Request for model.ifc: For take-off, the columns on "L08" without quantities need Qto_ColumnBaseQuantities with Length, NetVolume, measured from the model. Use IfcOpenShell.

First a look at what the model holds.

```python
import ifcopenshell
import ifcopenshell.util.element
import ifcopenshell.util.unit

model = ifcopenshell.open("model.ifc")
print(model.schema)
for unit_type in ("LENGTHUNIT", "AREAUNIT", "VOLUMEUNIT"):
    print(unit_type, ifcopenshell.util.unit.calculate_unit_scale(model, unit_type))
storey = next(s for s in model.by_type("IfcBuildingStorey") if s.Name == "L08")
columns = [e for e in ifcopenshell.util.element.get_decomposition(storey) if e.is_a("IfcColumn")]
for e in sorted(columns, key=lambda e: e.id()):
    print(e.id(), e.is_a(), e.Name, list(ifcopenshell.util.element.get_psets(e, qtos_only=True)), sep=" | ")
```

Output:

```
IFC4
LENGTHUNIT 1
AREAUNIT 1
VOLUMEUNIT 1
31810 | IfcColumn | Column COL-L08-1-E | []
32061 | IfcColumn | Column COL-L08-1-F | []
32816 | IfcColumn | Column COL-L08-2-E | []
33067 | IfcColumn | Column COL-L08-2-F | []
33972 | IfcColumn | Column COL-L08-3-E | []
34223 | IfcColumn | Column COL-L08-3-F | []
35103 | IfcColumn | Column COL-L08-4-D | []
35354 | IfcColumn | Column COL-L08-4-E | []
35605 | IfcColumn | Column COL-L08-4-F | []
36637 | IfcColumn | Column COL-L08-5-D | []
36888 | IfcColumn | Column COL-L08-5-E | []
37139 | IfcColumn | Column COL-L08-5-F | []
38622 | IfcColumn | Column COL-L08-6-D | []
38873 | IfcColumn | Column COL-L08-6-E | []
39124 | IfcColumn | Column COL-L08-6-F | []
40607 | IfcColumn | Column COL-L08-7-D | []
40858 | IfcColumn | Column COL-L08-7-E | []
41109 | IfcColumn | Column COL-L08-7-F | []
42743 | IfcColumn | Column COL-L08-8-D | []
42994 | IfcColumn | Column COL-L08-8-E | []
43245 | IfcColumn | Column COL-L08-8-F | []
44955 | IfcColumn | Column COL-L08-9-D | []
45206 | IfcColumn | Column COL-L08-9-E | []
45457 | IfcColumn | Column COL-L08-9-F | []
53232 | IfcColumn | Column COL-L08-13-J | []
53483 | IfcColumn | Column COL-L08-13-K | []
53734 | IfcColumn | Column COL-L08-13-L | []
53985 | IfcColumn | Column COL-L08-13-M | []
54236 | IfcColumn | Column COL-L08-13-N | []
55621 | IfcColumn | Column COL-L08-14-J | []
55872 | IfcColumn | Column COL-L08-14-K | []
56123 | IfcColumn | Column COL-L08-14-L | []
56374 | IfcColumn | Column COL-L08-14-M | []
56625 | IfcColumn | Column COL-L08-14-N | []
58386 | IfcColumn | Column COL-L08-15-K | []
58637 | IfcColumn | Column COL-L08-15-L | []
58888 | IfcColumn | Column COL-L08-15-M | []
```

```python
import ifcopenshell
import ifcopenshell.api.pset
import ifcopenshell.geom
import ifcopenshell.util.element
import ifcopenshell.util.shape
import ifcopenshell.util.unit

model = ifcopenshell.open("model.ifc")
unit_scale = ifcopenshell.util.unit.calculate_unit_scale(model)
volume_scale = ifcopenshell.util.unit.calculate_unit_scale(model, "VOLUMEUNIT")
settings = ifcopenshell.geom.settings()

storey = next(s for s in model.by_type("IfcBuildingStorey") if s.Name == "L08")
columns = [e for e in ifcopenshell.util.element.get_decomposition(storey) if e.is_a("IfcColumn")]

for e in sorted(columns, key=lambda e: e.id()):
    if ifcopenshell.util.element.get_psets(e, qtos_only=True, should_inherit=False):
        continue
    # Geometry comes back in metres, in the element's own axes.
    shape = ifcopenshell.geom.create_shape(settings, e)
    values = {
        "Length": ifcopenshell.util.shape.get_z(shape.geometry) / unit_scale,
        "NetVolume": ifcopenshell.util.shape.get_volume(shape.geometry) / volume_scale,
    }
    qto = ifcopenshell.api.pset.add_qto(model, product=e, name="Qto_ColumnBaseQuantities")
    ifcopenshell.api.pset.edit_qto(model, qto=qto, properties=values)
    print(e.id(), {k: round(v, 3) for k, v in values.items()})

model.write("model_v2.ifc")
```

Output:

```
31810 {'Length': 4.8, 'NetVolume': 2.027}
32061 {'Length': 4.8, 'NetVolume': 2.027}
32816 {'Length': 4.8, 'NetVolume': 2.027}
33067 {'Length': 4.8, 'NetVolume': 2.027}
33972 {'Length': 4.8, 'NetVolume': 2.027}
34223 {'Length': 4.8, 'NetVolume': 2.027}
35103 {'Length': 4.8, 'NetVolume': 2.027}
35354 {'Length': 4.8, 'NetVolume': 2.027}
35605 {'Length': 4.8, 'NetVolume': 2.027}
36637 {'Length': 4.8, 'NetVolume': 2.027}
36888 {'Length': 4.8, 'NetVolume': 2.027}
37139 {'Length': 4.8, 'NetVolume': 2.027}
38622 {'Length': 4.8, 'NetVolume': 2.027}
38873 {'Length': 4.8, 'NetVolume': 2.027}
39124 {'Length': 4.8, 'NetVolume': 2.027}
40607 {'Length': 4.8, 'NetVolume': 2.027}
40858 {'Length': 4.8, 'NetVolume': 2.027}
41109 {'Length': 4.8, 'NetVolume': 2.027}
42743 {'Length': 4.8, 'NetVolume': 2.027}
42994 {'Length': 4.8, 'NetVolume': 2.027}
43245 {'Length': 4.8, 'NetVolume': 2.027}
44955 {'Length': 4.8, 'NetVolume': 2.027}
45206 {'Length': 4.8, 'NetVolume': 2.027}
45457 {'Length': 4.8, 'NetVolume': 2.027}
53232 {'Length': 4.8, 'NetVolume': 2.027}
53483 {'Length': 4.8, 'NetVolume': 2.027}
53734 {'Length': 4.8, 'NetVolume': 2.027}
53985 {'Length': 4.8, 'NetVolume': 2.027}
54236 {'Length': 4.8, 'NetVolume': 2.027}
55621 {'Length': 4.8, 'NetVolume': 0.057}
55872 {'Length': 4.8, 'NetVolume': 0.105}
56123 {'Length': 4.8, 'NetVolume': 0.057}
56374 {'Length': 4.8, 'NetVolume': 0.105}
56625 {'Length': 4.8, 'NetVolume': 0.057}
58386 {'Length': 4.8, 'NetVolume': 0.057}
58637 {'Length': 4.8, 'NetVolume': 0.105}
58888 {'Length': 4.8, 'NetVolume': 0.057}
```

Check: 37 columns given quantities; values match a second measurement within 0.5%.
